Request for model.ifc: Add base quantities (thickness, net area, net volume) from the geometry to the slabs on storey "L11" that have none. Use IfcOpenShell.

First a look at what the model holds.

```python
import ifcopenshell
import ifcopenshell.util.element
import ifcopenshell.util.unit

model = ifcopenshell.open("model.ifc")
print(model.schema)
for unit_type in ("LENGTHUNIT", "AREAUNIT", "VOLUMEUNIT"):
    print(unit_type, ifcopenshell.util.unit.calculate_unit_scale(model, unit_type))
storey = next(s for s in model.by_type("IfcBuildingStorey") if s.Name == "L11")
slabs = [e for e in ifcopenshell.util.element.get_decomposition(storey) if e.is_a("IfcSlab")]
for e in sorted(slabs, key=lambda e: e.id()):
    print(e.id(), e.is_a(), e.Name, list(ifcopenshell.util.element.get_psets(e, qtos_only=True)), sep=" | ")
```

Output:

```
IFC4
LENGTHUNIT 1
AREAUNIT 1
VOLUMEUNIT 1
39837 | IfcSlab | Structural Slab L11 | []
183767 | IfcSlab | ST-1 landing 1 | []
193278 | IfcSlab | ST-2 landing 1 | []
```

```python
import ifcopenshell
import ifcopenshell.api.pset
import ifcopenshell.geom
import ifcopenshell.util.element
import ifcopenshell.util.shape
import ifcopenshell.util.unit

model = ifcopenshell.open("model.ifc")
unit_scale = ifcopenshell.util.unit.calculate_unit_scale(model)
area_scale = ifcopenshell.util.unit.calculate_unit_scale(model, "AREAUNIT")
volume_scale = ifcopenshell.util.unit.calculate_unit_scale(model, "VOLUMEUNIT")
settings = ifcopenshell.geom.settings()

storey = next(s for s in model.by_type("IfcBuildingStorey") if s.Name == "L11")
slabs = [e for e in ifcopenshell.util.element.get_decomposition(storey) if e.is_a("IfcSlab")]

for e in sorted(slabs, key=lambda e: e.id()):
    if ifcopenshell.util.element.get_psets(e, qtos_only=True, should_inherit=False):
        continue
    # Geometry comes back in metres, in the element's own axes.
    shape = ifcopenshell.geom.create_shape(settings, e)
    values = {
        "Width": ifcopenshell.util.shape.get_z(shape.geometry) / unit_scale,
        "NetArea": ifcopenshell.util.shape.get_footprint_area(shape.geometry) / area_scale,
        "NetVolume": ifcopenshell.util.shape.get_volume(shape.geometry) / volume_scale,
    }
    qto = ifcopenshell.api.pset.add_qto(model, product=e, name="Qto_SlabBaseQuantities")
    ifcopenshell.api.pset.edit_qto(model, qto=qto, properties=values)
    print(e.id(), {k: round(v, 3) for k, v in values.items()})

model.write("model_edited.ifc")
```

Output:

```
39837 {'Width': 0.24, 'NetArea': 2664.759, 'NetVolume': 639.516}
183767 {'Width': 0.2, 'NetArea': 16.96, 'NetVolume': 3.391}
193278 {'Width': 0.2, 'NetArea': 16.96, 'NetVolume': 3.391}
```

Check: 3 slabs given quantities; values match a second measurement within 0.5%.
